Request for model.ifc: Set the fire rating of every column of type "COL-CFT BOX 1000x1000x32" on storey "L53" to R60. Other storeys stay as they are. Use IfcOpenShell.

First a look at what the model holds.

```python
import ifcopenshell
import ifcopenshell.util.element

model = ifcopenshell.open("model.ifc")
print(model.schema)
storey = next(s for s in model.by_type("IfcBuildingStorey") if s.Name == "L53")
columns = [e for e in ifcopenshell.util.element.get_decomposition(storey) if e.is_a("IfcColumn")]
seen = {}
for e in columns:
    element_type = ifcopenshell.util.element.get_type(e)
    key = (element_type.Name if element_type != e and element_type else None, ifcopenshell.util.element.get_pset(e, "Pset_ColumnCommon", "FireRating"))
    seen[key] = seen.get(key, 0) + 1
for (name, value), count in sorted(seen.items(), key=str):
    print(count, "x", name, "|", value)
```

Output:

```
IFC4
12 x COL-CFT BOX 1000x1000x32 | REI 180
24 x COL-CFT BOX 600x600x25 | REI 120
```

```python
import ifcopenshell
import ifcopenshell.api.pset
import ifcopenshell.util.element

model = ifcopenshell.open("model.ifc")

storey = next(s for s in model.by_type("IfcBuildingStorey") if s.Name == "L53")
columns = [e for e in ifcopenshell.util.element.get_decomposition(storey) if e.is_a("IfcColumn")]

count = 0
for e in columns:
    element_type = ifcopenshell.util.element.get_type(e)
    if element_type in (None, e) or element_type.Name != "COL-CFT BOX 1000x1000x32":
        continue
    # add_pset returns the element's existing set when there is one.
    pset = ifcopenshell.api.pset.add_pset(model, product=e, name="Pset_ColumnCommon")
    ifcopenshell.api.pset.edit_pset(model, pset=pset, properties={"FireRating": "R60"})
    count += 1

print(count, "columns updated")

model.write("model_rev.ifc")
```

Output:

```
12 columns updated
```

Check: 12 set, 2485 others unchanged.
